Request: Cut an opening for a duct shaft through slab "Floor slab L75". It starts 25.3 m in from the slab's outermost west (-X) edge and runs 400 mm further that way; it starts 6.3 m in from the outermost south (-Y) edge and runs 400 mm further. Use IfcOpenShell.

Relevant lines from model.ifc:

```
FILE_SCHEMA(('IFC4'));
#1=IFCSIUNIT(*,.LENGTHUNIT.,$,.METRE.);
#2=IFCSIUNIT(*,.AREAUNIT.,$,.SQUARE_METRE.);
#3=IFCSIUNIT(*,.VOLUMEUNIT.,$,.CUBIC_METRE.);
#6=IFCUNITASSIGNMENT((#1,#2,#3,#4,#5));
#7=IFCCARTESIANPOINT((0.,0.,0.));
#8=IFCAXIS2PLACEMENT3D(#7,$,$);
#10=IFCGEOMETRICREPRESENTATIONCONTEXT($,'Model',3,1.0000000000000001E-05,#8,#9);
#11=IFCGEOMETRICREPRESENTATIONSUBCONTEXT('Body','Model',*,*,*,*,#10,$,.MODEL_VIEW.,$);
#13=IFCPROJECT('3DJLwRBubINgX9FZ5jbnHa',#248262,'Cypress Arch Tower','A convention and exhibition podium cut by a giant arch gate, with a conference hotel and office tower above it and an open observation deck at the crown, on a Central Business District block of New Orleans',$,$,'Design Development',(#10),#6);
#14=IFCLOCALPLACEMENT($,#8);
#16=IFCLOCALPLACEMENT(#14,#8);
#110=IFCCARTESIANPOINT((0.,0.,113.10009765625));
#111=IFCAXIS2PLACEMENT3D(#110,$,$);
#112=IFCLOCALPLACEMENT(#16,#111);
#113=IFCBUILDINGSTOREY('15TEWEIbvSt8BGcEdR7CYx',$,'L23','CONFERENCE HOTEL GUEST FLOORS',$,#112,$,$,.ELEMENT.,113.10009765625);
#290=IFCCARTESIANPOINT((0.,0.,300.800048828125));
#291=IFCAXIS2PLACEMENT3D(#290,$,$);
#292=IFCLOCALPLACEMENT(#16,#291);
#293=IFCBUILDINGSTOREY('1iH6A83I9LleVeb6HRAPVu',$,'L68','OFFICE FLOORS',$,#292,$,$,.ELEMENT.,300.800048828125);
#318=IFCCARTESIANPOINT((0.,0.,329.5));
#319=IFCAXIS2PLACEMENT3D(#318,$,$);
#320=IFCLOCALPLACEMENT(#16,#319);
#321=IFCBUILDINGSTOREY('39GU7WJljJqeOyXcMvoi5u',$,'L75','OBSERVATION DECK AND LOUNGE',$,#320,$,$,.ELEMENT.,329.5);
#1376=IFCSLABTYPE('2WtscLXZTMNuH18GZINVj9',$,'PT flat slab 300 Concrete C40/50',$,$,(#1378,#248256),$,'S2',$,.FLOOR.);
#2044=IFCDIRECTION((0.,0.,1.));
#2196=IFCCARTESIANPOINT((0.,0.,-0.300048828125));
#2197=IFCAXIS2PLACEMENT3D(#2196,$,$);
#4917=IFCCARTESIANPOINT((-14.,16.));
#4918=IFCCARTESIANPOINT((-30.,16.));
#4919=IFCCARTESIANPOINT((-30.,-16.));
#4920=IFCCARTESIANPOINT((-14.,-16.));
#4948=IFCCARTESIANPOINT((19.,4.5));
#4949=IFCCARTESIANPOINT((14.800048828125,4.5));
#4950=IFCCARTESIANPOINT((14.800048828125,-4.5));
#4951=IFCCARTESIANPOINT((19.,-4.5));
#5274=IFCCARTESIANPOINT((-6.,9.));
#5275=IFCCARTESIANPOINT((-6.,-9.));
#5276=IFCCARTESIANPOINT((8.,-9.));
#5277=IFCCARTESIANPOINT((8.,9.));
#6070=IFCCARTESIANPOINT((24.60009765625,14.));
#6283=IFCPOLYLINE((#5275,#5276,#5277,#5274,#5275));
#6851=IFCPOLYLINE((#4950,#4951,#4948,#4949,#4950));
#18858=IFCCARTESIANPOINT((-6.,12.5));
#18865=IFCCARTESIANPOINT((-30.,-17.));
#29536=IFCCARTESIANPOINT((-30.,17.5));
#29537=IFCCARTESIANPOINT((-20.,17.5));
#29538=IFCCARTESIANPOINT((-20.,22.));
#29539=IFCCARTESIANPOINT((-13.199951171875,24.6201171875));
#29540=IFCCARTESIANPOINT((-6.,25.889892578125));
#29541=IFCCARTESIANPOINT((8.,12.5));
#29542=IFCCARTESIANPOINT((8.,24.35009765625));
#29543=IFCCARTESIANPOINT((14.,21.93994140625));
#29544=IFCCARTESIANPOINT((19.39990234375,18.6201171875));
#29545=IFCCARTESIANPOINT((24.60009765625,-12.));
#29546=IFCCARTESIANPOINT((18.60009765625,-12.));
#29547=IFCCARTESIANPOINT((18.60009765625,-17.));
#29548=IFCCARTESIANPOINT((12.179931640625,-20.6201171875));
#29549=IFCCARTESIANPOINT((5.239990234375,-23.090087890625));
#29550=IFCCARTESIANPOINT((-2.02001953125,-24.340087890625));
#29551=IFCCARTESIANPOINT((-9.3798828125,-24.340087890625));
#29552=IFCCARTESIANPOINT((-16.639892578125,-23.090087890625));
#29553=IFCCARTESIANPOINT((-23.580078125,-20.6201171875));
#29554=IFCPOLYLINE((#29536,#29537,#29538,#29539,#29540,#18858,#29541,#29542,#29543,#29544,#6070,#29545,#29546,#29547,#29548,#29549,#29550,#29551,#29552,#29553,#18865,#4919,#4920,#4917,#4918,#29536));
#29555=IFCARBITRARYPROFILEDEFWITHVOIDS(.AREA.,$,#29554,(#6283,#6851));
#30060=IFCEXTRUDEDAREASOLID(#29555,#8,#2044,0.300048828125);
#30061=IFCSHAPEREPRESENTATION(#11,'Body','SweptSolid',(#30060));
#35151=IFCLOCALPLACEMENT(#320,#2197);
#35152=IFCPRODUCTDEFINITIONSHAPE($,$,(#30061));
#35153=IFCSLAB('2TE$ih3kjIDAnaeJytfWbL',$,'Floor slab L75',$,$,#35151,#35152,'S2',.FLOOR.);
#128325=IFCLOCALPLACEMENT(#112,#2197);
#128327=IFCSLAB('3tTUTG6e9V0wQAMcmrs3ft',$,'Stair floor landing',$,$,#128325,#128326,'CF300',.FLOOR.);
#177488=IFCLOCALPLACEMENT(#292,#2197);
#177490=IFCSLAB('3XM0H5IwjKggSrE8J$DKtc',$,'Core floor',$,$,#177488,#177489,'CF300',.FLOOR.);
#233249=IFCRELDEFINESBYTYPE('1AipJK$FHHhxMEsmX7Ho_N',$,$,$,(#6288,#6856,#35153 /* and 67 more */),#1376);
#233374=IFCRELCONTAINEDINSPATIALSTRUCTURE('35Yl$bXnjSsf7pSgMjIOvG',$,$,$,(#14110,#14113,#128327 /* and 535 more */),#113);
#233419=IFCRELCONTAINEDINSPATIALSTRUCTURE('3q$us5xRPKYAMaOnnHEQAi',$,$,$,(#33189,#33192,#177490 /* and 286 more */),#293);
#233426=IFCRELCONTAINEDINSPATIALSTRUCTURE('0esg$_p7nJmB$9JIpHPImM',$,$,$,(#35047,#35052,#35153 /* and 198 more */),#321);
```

```python
import numpy as np
import ifcopenshell
import ifcopenshell.api.feature
import ifcopenshell.api.geometry
import ifcopenshell.api.root
import ifcopenshell.geom
import ifcopenshell.util.placement
import ifcopenshell.util.representation
import ifcopenshell.util.shape
import ifcopenshell.util.unit

model = ifcopenshell.open("model.ifc")
unit_scale = ifcopenshell.util.unit.calculate_unit_scale(model)
settings = ifcopenshell.geom.settings()


def volume(element):
    """Net volume in cubic metres, openings subtracted."""
    shape = ifcopenshell.geom.create_shape(settings, element)
    return ifcopenshell.util.shape.get_volume(shape.geometry)


slab = model.by_guid("2TE$ih3kjIDAnaeJytfWbL")
before = volume(slab)

# Extent in the slab's own axes, in metres. The edges named are its -X and -Y sides.
slab_shape = ifcopenshell.geom.create_shape(settings, slab)
vertices = ifcopenshell.util.shape.get_vertices(slab_shape.geometry)
x_min, y_min, bottom = vertices.min(axis=0)
top = vertices[:, 2].max()

opening = ifcopenshell.api.root.create_entity(model, ifc_class="IfcOpeningElement", name="Duct shaft opening", predefined_type="OPENING")
context = ifcopenshell.util.representation.get_context(model, "Model", "Body", "MODEL_VIEW")
width, depth = 0.4, 0.4
outline = [(0.0, 0.0), (width, 0.0), (width, depth), (0.0, depth), (0.0, 0.0)]
# Overshoot both faces by 50 mm so the cut is clean.
shape = ifcopenshell.api.geometry.add_slab_representation(
    model, context=context, depth=top - bottom + 0.1, polyline=outline
)
ifcopenshell.api.geometry.assign_representation(model, product=opening, representation=shape)

matrix = ifcopenshell.util.placement.get_local_placement(slab.ObjectPlacement)
matrix[:, 3] = matrix @ np.append(np.array([x_min + 25.3, y_min + 6.3, bottom - 0.05]) / unit_scale, 1.0)
ifcopenshell.api.geometry.edit_object_placement(model, product=opening, matrix=matrix, is_si=False)
ifcopenshell.api.feature.add_feature(model, feature=opening, element=slab)

after = volume(slab)

print(f"slab volume {before:.3f} -> {after:.3f} m3")

model.write("model_updated.ifc")
```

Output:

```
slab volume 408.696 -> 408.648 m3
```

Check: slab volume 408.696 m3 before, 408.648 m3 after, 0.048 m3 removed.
